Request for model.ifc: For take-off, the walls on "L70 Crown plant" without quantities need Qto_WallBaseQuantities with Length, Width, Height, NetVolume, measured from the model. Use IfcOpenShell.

First a look at what the model holds.

```python
import ifcopenshell
import ifcopenshell.util.element
import ifcopenshell.util.unit

model = ifcopenshell.open("model.ifc")
print(model.schema)
for unit_type in ("LENGTHUNIT", "AREAUNIT", "VOLUMEUNIT"):
    print(unit_type, ifcopenshell.util.unit.calculate_unit_scale(model, unit_type))
storey = next(s for s in model.by_type("IfcBuildingStorey") if s.Name == "L70 Crown plant")
walls = [e for e in ifcopenshell.util.element.get_decomposition(storey) if e.is_a("IfcWall")]
for e in sorted(walls, key=lambda e: e.id()):
    print(e.id(), e.is_a(), e.Name, list(ifcopenshell.util.element.get_psets(e, qtos_only=True)), sep=" | ")
```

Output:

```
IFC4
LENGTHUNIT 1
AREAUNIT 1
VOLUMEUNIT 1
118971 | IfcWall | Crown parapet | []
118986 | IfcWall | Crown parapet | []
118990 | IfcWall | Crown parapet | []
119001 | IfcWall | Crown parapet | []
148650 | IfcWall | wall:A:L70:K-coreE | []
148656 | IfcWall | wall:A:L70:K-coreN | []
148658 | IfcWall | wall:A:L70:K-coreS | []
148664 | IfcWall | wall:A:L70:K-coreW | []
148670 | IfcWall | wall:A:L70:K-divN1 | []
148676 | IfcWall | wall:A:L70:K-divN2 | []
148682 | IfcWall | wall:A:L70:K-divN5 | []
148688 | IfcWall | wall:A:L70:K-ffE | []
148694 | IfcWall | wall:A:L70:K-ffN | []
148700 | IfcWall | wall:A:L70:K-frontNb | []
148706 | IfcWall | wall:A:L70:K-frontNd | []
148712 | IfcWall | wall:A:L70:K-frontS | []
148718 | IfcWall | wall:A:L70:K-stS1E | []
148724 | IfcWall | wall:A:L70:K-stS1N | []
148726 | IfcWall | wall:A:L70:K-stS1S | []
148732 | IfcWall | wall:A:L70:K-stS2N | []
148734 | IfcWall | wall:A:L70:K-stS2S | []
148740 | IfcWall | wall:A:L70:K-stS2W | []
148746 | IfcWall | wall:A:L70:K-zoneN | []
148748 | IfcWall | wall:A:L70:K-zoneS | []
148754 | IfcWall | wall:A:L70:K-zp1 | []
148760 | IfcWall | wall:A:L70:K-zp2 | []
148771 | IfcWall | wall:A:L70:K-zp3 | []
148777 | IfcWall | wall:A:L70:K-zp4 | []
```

```python
import ifcopenshell
import ifcopenshell.api.pset
import ifcopenshell.geom
import ifcopenshell.util.element
import ifcopenshell.util.shape
import ifcopenshell.util.unit

model = ifcopenshell.open("model.ifc")
unit_scale = ifcopenshell.util.unit.calculate_unit_scale(model)
volume_scale = ifcopenshell.util.unit.calculate_unit_scale(model, "VOLUMEUNIT")
settings = ifcopenshell.geom.settings()

storey = next(s for s in model.by_type("IfcBuildingStorey") if s.Name == "L70 Crown plant")
walls = [e for e in ifcopenshell.util.element.get_decomposition(storey) if e.is_a("IfcWall")]

for e in sorted(walls, key=lambda e: e.id()):
    if ifcopenshell.util.element.get_psets(e, qtos_only=True, should_inherit=False):
        continue
    # Geometry comes back in metres, in the element's own axes.
    shape = ifcopenshell.geom.create_shape(settings, e)
    values = {
        "Length": ifcopenshell.util.shape.get_x(shape.geometry) / unit_scale,
        "Width": ifcopenshell.util.shape.get_y(shape.geometry) / unit_scale,
        "Height": ifcopenshell.util.shape.get_z(shape.geometry) / unit_scale,
        "NetVolume": ifcopenshell.util.shape.get_volume(shape.geometry) / volume_scale,
    }
    qto = ifcopenshell.api.pset.add_qto(model, product=e, name="Qto_WallBaseQuantities")
    ifcopenshell.api.pset.edit_qto(model, qto=qto, properties=values)
    print(e.id(), {k: round(v, 3) for k, v in values.items()})

model.write("model_updated.ifc")
```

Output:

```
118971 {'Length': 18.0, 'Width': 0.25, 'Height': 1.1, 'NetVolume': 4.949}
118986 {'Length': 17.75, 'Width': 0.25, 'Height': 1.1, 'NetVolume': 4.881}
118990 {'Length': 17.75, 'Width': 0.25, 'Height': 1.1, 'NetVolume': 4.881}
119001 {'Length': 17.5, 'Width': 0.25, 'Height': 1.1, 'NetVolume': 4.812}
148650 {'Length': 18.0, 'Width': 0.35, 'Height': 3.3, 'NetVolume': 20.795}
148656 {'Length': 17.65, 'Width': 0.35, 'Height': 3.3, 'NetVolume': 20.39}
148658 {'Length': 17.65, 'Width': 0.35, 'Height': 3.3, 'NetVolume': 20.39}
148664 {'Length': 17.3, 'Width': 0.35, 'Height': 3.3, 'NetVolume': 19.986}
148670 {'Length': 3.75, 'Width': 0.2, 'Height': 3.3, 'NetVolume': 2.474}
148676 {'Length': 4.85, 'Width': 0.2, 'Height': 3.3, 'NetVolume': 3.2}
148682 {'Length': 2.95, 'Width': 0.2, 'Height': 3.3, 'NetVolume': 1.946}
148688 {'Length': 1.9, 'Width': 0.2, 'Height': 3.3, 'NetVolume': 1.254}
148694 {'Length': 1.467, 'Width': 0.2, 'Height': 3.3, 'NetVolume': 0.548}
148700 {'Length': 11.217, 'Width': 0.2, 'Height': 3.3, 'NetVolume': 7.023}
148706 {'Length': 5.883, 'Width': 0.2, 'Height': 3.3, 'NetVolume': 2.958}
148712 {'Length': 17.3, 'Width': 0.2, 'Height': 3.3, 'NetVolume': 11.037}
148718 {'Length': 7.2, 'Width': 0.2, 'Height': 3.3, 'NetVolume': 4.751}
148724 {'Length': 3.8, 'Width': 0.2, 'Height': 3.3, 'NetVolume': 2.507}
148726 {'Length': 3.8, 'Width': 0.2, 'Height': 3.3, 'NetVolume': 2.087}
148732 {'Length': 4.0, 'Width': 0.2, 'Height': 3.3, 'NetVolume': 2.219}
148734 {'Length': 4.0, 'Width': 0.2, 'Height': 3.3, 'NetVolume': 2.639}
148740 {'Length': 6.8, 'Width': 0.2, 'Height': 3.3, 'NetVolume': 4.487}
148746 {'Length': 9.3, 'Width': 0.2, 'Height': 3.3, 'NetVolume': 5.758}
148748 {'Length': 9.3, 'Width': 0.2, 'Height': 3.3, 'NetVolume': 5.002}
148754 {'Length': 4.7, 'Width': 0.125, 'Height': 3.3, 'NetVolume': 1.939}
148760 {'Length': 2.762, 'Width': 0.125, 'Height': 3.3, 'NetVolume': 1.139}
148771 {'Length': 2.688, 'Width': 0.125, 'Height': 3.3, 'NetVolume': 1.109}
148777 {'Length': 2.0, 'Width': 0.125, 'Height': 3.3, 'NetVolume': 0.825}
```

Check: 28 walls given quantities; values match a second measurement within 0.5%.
